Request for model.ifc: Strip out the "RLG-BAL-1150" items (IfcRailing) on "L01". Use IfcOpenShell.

First a look at what the model holds.

```python
import ifcopenshell
import ifcopenshell.util.element

model = ifcopenshell.open("model.ifc")
print(model.schema)
storey = next(s for s in model.by_type("IfcBuildingStorey") if s.Name == "L01")
railings = [e for e in ifcopenshell.util.element.get_decomposition(storey) if e.is_a("IfcRailing")]
seen = {}
for e in railings:
    element_type = ifcopenshell.util.element.get_type(e)
    name = element_type.Name if element_type not in (None, e) else None
    seen[name] = seen.get(name, 0) + 1
for name, count in sorted(seen.items(), key=str):
    print(count, "x", name)
```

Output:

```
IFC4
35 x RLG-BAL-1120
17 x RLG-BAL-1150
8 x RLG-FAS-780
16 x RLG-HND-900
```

```python
import ifcopenshell
import ifcopenshell.api.root
import ifcopenshell.util.element

model = ifcopenshell.open("model.ifc")

storey = next(s for s in model.by_type("IfcBuildingStorey") if s.Name == "L01")
railings = [e for e in ifcopenshell.util.element.get_decomposition(storey) if e.is_a("IfcRailing")]
targets = [e for e in railings if (t := ifcopenshell.util.element.get_type(e)) not in (None, e) and t.Name == "RLG-BAL-1150"]

for e in targets:
    ifcopenshell.api.root.remove_product(model, product=e)
print(len(targets), "removed")

model.write("model_v2.ifc")
```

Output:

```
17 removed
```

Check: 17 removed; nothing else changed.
